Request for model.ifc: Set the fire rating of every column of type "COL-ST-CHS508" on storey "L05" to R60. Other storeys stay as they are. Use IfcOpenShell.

First a look at what the model holds.

```python
import ifcopenshell
import ifcopenshell.util.element

model = ifcopenshell.open("model.ifc")
print(model.schema)
storey = next(s for s in model.by_type("IfcBuildingStorey") if s.Name == "L05")
columns = [e for e in ifcopenshell.util.element.get_decomposition(storey) if e.is_a("IfcColumn")]
seen = {}
for e in columns:
    element_type = ifcopenshell.util.element.get_type(e)
    key = (element_type.Name if element_type != e and element_type else None, ifcopenshell.util.element.get_pset(e, "Pset_ColumnCommon", "FireRating"))
    seen[key] = seen.get(key, 0) + 1
for (name, value), count in sorted(seen.items(), key=str):
    print(count, "x", name, "|", value)
```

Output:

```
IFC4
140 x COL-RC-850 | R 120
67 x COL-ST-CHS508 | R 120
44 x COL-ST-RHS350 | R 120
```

```python
import ifcopenshell
import ifcopenshell.api.pset
import ifcopenshell.util.element

model = ifcopenshell.open("model.ifc")

storey = next(s for s in model.by_type("IfcBuildingStorey") if s.Name == "L05")
columns = [e for e in ifcopenshell.util.element.get_decomposition(storey) if e.is_a("IfcColumn")]

count = 0
for e in columns:
    element_type = ifcopenshell.util.element.get_type(e)
    if element_type in (None, e) or element_type.Name != "COL-ST-CHS508":
        continue
    # add_pset returns the element's existing set when there is one.
    pset = ifcopenshell.api.pset.add_pset(model, product=e, name="Pset_ColumnCommon")
    ifcopenshell.api.pset.edit_pset(model, pset=pset, properties={"FireRating": "R60"})
    count += 1

print(count, "columns updated")

model.write("model_updated.ifc")
```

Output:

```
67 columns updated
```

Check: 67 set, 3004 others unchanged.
